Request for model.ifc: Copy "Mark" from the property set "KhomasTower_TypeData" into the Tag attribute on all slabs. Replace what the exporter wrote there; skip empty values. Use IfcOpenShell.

First a look at what the model holds.

```python
import ifcopenshell
import ifcopenshell.util.element

model = ifcopenshell.open("model.ifc")
print(model.schema)
slabs = model.by_type("IfcSlab")
print(len(slabs), "slabs")
for e in slabs[:8]:
    source = ifcopenshell.util.element.get_pset(e, "KhomasTower_TypeData", "Mark")
    target = e.Tag
    print(e.id(), repr(source), repr(target), sep=" | ")
```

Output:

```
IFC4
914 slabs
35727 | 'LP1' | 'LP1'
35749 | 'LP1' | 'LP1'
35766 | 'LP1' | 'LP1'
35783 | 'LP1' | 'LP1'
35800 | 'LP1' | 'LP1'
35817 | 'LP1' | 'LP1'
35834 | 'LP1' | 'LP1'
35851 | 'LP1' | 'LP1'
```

```python
import ifcopenshell
import ifcopenshell.util.element

model = ifcopenshell.open("model.ifc")

count = 0
for e in model.by_type("IfcSlab"):
    value = ifcopenshell.util.element.get_pset(e, "KhomasTower_TypeData", "Mark")
    current = e.Tag
    if not value or not value.strip() or current == value:
        continue
    e.Tag = value
    count += 1

print(count, "slabs updated")

model.write("model_edited.ifc")
```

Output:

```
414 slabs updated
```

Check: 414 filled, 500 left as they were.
